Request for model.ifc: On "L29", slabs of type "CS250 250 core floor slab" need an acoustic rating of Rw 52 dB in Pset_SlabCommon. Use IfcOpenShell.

First a look at what the model holds.

```python
import ifcopenshell
import ifcopenshell.util.element

model = ifcopenshell.open("model.ifc")
print(model.schema)
storey = next(s for s in model.by_type("IfcBuildingStorey") if s.Name == "L29")
slabs = [e for e in ifcopenshell.util.element.get_decomposition(storey) if e.is_a("IfcSlab")]
seen = {}
for e in slabs:
    element_type = ifcopenshell.util.element.get_type(e)
    key = (element_type.Name if element_type != e and element_type else None, ifcopenshell.util.element.get_pset(e, "Pset_SlabCommon", "AcousticRating"))
    seen[key] = seen.get(key, 0) + 1
for (name, value), count in sorted(seen.items(), key=str):
    print(count, "x", name, "|", value)
```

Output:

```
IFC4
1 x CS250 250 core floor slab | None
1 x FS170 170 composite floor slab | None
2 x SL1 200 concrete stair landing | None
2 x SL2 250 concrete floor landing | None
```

```python
import ifcopenshell
import ifcopenshell.api.pset
import ifcopenshell.util.element

model = ifcopenshell.open("model.ifc")

storey = next(s for s in model.by_type("IfcBuildingStorey") if s.Name == "L29")
slabs = [e for e in ifcopenshell.util.element.get_decomposition(storey) if e.is_a("IfcSlab")]

count = 0
for e in slabs:
    element_type = ifcopenshell.util.element.get_type(e)
    if element_type in (None, e) or element_type.Name != "CS250 250 core floor slab":
        continue
    # add_pset returns the element's existing set when there is one.
    pset = ifcopenshell.api.pset.add_pset(model, product=e, name="Pset_SlabCommon")
    ifcopenshell.api.pset.edit_pset(model, pset=pset, properties={"AcousticRating": "Rw 52 dB"})
    count += 1

print(count, "slabs updated")

model.write("model_updated.ifc")
```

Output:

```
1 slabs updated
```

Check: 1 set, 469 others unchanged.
